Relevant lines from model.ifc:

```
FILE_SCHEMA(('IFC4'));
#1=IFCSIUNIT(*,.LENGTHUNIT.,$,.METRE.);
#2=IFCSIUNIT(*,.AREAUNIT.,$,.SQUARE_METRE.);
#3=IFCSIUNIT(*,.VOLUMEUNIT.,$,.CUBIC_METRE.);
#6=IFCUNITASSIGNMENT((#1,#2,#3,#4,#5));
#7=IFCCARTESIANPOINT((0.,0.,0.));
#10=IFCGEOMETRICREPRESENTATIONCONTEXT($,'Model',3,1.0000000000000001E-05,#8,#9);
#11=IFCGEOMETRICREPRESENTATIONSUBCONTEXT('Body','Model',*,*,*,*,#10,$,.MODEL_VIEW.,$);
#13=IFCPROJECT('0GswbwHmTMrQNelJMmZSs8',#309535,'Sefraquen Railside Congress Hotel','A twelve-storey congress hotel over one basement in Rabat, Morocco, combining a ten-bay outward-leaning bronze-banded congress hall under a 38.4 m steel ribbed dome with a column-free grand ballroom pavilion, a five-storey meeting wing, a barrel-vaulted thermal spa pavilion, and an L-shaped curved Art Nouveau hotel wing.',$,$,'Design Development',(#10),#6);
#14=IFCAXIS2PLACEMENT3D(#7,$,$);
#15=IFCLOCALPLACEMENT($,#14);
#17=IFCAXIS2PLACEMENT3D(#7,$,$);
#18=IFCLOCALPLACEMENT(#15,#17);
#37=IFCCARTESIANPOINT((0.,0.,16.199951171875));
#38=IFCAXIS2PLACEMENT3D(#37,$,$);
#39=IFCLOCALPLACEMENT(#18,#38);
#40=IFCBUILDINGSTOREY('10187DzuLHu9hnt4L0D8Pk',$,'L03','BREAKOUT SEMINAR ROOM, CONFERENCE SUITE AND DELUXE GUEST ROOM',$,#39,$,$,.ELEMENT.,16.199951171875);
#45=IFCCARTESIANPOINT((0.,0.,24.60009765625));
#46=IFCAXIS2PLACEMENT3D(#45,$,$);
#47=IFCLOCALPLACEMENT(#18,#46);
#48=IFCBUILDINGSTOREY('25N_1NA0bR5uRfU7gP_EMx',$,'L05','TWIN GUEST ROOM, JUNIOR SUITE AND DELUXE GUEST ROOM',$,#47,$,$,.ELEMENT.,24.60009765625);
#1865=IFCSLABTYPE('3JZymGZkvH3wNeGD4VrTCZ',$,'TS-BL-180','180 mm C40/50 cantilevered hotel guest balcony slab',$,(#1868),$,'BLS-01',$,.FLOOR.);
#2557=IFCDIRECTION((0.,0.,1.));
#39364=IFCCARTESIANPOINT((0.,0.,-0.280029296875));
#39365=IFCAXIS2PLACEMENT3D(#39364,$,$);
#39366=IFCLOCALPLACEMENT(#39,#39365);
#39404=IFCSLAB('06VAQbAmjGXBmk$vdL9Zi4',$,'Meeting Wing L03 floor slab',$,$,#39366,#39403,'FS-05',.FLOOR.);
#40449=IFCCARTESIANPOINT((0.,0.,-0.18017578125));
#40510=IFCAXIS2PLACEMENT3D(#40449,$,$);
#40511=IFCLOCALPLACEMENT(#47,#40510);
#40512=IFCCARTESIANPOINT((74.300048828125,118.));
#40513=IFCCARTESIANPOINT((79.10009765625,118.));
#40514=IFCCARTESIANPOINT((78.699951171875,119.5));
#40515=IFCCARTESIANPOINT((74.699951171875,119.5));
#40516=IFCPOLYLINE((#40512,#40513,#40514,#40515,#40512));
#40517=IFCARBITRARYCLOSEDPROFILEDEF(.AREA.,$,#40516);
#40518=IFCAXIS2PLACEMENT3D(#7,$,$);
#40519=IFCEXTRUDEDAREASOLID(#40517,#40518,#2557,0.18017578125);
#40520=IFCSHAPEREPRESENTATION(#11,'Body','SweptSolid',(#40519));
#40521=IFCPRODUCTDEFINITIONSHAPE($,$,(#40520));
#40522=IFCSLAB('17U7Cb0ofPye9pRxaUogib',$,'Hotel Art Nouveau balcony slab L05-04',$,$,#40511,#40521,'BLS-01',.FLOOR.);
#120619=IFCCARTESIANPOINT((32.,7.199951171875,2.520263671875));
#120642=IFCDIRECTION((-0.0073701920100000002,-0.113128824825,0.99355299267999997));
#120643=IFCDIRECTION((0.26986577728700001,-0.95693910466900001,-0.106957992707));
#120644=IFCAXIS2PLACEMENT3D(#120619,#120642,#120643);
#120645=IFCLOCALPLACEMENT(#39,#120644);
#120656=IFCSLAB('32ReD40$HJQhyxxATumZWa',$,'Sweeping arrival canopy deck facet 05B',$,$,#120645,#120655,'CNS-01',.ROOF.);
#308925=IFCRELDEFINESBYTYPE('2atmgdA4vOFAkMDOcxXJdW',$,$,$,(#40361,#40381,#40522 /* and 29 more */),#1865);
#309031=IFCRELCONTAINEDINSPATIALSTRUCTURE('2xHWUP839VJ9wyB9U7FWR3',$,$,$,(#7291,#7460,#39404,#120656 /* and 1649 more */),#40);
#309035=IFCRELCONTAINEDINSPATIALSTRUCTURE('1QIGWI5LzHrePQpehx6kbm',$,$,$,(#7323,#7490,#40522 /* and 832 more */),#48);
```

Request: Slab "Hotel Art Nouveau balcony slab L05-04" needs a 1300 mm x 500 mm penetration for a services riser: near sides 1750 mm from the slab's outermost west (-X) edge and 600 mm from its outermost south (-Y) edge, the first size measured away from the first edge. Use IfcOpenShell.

```python
import numpy as np
import ifcopenshell
import ifcopenshell.api.feature
import ifcopenshell.api.geometry
import ifcopenshell.api.root
import ifcopenshell.geom
import ifcopenshell.util.placement
import ifcopenshell.util.representation
import ifcopenshell.util.shape
import ifcopenshell.util.unit

model = ifcopenshell.open("model.ifc")
unit_scale = ifcopenshell.util.unit.calculate_unit_scale(model)
settings = ifcopenshell.geom.settings()


def volume(element):
    """Net volume in cubic metres, openings subtracted."""
    shape = ifcopenshell.geom.create_shape(settings, element)
    return ifcopenshell.util.shape.get_volume(shape.geometry)


slab = model.by_guid("17U7Cb0ofPye9pRxaUogib")
before = volume(slab)

# Extent in the slab's own axes, in metres. The edges named are its -X and -Y sides.
slab_shape = ifcopenshell.geom.create_shape(settings, slab)
vertices = ifcopenshell.util.shape.get_vertices(slab_shape.geometry)
x_min, y_min, bottom = vertices.min(axis=0)
top = vertices[:, 2].max()

opening = ifcopenshell.api.root.create_entity(model, ifc_class="IfcOpeningElement", name="Services riser opening", predefined_type="OPENING")
context = ifcopenshell.util.representation.get_context(model, "Model", "Body", "MODEL_VIEW")
width, depth = 1.3, 0.5
outline = [(0.0, 0.0), (width, 0.0), (width, depth), (0.0, depth), (0.0, 0.0)]
# Overshoot both faces by 50 mm so the cut is clean.
shape = ifcopenshell.api.geometry.add_slab_representation(
    model, context=context, depth=top - bottom + 0.1, polyline=outline
)
ifcopenshell.api.geometry.assign_representation(model, product=opening, representation=shape)

matrix = ifcopenshell.util.placement.get_local_placement(slab.ObjectPlacement)
matrix[:, 3] = matrix @ np.append(np.array([x_min + 1.75, y_min + 0.6, bottom - 0.05]) / unit_scale, 1.0)
ifcopenshell.api.geometry.edit_object_placement(model, product=opening, matrix=matrix, is_si=False)
ifcopenshell.api.feature.add_feature(model, feature=opening, element=slab)

after = volume(slab)

print(f"slab volume {before:.3f} -> {after:.3f} m3")

model.write("model_v2.ifc")
```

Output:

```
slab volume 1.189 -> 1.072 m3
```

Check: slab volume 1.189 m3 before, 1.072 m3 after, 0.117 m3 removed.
